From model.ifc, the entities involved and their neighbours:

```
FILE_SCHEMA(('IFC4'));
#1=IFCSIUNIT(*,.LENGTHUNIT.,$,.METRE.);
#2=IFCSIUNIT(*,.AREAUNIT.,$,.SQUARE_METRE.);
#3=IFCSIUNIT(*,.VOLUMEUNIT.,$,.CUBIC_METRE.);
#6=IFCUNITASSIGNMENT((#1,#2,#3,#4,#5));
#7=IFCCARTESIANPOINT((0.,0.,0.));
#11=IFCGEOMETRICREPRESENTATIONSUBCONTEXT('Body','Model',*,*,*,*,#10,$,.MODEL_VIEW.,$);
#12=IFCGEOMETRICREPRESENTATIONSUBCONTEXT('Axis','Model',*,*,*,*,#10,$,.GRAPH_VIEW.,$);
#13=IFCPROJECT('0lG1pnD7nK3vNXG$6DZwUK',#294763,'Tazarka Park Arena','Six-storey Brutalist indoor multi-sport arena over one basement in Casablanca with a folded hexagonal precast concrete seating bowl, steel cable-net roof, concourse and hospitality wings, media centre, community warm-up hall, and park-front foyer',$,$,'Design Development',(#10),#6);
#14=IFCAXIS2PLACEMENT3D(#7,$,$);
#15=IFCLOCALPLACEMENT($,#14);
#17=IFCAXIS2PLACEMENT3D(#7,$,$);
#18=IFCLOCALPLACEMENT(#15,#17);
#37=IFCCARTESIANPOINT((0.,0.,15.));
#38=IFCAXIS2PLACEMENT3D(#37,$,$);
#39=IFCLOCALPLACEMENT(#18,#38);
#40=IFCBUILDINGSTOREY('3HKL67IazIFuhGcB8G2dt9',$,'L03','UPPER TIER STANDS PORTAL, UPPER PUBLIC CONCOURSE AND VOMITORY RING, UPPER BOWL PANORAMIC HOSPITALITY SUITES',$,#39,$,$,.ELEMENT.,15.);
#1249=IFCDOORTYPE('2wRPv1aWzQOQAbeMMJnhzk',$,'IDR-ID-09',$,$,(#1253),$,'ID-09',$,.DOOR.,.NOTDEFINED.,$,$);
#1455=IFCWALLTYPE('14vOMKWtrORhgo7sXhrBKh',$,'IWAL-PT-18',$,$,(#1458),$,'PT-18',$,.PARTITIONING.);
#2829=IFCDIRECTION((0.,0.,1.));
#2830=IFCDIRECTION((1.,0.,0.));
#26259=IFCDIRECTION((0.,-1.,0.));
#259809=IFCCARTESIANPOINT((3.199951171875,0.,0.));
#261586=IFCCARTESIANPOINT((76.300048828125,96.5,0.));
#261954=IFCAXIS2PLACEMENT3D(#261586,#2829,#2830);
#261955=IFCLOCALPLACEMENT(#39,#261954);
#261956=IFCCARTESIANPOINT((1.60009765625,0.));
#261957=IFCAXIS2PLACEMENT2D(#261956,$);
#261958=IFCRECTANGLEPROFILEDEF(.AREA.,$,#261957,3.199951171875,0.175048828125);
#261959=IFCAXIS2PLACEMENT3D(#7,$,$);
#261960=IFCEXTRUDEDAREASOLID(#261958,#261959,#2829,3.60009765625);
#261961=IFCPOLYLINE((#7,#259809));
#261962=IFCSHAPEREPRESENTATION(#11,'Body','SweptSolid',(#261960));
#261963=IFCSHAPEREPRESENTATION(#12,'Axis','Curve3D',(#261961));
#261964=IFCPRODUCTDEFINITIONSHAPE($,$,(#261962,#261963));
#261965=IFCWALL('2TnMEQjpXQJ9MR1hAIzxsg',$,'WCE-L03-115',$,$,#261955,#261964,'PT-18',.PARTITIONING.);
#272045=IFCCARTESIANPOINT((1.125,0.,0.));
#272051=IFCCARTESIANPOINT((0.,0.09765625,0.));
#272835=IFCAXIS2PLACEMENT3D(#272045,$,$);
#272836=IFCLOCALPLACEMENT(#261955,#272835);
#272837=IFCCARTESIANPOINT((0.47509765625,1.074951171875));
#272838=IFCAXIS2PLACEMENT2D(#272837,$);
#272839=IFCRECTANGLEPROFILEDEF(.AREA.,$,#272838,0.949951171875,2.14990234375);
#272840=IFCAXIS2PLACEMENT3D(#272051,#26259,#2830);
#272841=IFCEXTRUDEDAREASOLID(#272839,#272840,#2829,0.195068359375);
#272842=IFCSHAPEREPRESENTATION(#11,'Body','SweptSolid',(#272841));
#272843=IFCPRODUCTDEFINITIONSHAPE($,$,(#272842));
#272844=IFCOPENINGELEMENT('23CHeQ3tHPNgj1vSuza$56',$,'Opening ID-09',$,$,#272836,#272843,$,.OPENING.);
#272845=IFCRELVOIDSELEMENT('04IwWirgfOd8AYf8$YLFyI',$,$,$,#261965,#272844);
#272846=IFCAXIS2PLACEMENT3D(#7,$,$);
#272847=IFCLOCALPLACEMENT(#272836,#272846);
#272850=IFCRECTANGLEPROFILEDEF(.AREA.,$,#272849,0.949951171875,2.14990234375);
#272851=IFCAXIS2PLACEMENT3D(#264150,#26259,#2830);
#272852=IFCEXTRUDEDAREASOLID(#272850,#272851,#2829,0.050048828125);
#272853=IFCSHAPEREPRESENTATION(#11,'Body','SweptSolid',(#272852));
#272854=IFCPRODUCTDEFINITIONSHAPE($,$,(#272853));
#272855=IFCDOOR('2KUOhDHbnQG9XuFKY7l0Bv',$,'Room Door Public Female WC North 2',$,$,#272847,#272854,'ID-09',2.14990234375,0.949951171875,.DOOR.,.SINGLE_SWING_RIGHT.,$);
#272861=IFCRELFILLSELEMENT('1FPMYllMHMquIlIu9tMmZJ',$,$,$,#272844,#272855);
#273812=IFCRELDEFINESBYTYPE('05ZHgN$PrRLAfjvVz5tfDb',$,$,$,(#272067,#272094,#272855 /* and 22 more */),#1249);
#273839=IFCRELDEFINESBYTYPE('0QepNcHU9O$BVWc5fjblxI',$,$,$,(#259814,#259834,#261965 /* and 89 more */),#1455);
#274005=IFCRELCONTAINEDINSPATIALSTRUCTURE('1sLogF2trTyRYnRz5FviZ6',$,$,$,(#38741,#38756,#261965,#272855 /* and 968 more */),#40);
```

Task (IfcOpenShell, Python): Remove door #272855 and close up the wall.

```python
import ifcopenshell
import ifcopenshell.api.feature
import ifcopenshell.api.root
import ifcopenshell.geom
import ifcopenshell.util.shape

model = ifcopenshell.open("model.ifc")
settings = ifcopenshell.geom.settings()


def volume(element):
    """Net volume in cubic metres, openings subtracted."""
    shape = ifcopenshell.geom.create_shape(settings, element)
    return ifcopenshell.util.shape.get_volume(shape.geometry)


door = model.by_guid("2KUOhDHbnQG9XuFKY7l0Bv")
opening = door.FillsVoids[0].RelatingOpeningElement
wall = opening.VoidsElements[0].RelatingBuildingElement
before = volume(wall)

ifcopenshell.api.root.remove_product(model, product=door)
ifcopenshell.api.feature.remove_feature(model, feature=opening)

after = volume(wall)

print(f"wall volume {before:.3f} -> {after:.3f} m3")

model.write("model_edited.ifc")
```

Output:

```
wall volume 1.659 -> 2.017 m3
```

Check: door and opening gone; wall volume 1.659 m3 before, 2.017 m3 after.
